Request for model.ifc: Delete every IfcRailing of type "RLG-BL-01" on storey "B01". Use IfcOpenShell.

First a look at what the model holds.

```python
import ifcopenshell
import ifcopenshell.util.element

model = ifcopenshell.open("model.ifc")
print(model.schema)
storey = next(s for s in model.by_type("IfcBuildingStorey") if s.Name == "B01")
railings = [e for e in ifcopenshell.util.element.get_decomposition(storey) if e.is_a("IfcRailing")]
seen = {}
for e in railings:
    element_type = ifcopenshell.util.element.get_type(e)
    name = element_type.Name if element_type not in (None, e) else None
    seen[name] = seen.get(name, 0) + 1
for name, count in sorted(seen.items(), key=str):
    print(count, "x", name)
```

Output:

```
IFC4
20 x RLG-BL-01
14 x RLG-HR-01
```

```python
import ifcopenshell
import ifcopenshell.api.root
import ifcopenshell.util.element

model = ifcopenshell.open("model.ifc")

storey = next(s for s in model.by_type("IfcBuildingStorey") if s.Name == "B01")
railings = [e for e in ifcopenshell.util.element.get_decomposition(storey) if e.is_a("IfcRailing")]
targets = [e for e in railings if (t := ifcopenshell.util.element.get_type(e)) not in (None, e) and t.Name == "RLG-BL-01"]

for e in targets:
    ifcopenshell.api.root.remove_product(model, product=e)
print(len(targets), "removed")

model.write("model_v2.ifc")
```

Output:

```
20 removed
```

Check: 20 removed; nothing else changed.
